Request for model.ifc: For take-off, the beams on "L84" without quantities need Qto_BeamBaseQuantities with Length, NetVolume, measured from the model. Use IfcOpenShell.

First a look at what the model holds.

```python
import ifcopenshell
import ifcopenshell.util.element
import ifcopenshell.util.unit

model = ifcopenshell.open("model.ifc")
print(model.schema)
for unit_type in ("LENGTHUNIT", "AREAUNIT", "VOLUMEUNIT"):
    print(unit_type, ifcopenshell.util.unit.calculate_unit_scale(model, unit_type))
storey = next(s for s in model.by_type("IfcBuildingStorey") if s.Name == "L84")
beams = [e for e in ifcopenshell.util.element.get_decomposition(storey) if e.is_a("IfcBeam")]
for e in sorted(beams, key=lambda e: e.id()):
    print(e.id(), e.is_a(), e.Name, list(ifcopenshell.util.element.get_psets(e, qtos_only=True)), sep=" | ")
```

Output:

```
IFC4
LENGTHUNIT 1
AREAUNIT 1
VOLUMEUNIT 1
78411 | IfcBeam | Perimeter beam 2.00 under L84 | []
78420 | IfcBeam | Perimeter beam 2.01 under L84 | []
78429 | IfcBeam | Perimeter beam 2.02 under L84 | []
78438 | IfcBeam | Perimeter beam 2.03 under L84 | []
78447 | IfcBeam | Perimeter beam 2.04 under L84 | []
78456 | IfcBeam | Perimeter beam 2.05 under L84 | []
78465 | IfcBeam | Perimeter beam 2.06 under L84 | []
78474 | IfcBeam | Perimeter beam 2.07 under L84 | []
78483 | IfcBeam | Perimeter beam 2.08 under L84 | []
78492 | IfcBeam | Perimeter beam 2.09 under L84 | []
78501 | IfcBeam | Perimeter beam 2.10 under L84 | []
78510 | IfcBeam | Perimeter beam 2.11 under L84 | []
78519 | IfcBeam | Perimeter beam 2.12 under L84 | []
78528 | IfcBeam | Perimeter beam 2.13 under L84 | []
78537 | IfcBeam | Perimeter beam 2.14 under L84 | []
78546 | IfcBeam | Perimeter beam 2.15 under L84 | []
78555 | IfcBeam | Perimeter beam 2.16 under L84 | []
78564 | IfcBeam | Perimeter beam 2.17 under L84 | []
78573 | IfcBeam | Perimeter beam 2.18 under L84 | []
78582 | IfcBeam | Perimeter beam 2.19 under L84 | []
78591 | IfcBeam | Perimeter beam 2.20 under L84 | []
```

```python
import ifcopenshell
import ifcopenshell.api.pset
import ifcopenshell.geom
import ifcopenshell.util.element
import ifcopenshell.util.shape
import ifcopenshell.util.unit

model = ifcopenshell.open("model.ifc")
unit_scale = ifcopenshell.util.unit.calculate_unit_scale(model)
volume_scale = ifcopenshell.util.unit.calculate_unit_scale(model, "VOLUMEUNIT")
settings = ifcopenshell.geom.settings()

storey = next(s for s in model.by_type("IfcBuildingStorey") if s.Name == "L84")
beams = [e for e in ifcopenshell.util.element.get_decomposition(storey) if e.is_a("IfcBeam")]

for e in sorted(beams, key=lambda e: e.id()):
    if ifcopenshell.util.element.get_psets(e, qtos_only=True, should_inherit=False):
        continue
    # Geometry comes back in metres, in the element's own axes.
    shape = ifcopenshell.geom.create_shape(settings, e)
    values = {
        "Length": ifcopenshell.util.shape.get_max_xyz(shape.geometry) / unit_scale,
        "NetVolume": ifcopenshell.util.shape.get_volume(shape.geometry) / volume_scale,
    }
    qto = ifcopenshell.api.pset.add_qto(model, product=e, name="Qto_BeamBaseQuantities")
    ifcopenshell.api.pset.edit_qto(model, qto=qto, properties=values)
    print(e.id(), {k: round(v, 3) for k, v in values.items()})

model.write("model_updated.ifc")
```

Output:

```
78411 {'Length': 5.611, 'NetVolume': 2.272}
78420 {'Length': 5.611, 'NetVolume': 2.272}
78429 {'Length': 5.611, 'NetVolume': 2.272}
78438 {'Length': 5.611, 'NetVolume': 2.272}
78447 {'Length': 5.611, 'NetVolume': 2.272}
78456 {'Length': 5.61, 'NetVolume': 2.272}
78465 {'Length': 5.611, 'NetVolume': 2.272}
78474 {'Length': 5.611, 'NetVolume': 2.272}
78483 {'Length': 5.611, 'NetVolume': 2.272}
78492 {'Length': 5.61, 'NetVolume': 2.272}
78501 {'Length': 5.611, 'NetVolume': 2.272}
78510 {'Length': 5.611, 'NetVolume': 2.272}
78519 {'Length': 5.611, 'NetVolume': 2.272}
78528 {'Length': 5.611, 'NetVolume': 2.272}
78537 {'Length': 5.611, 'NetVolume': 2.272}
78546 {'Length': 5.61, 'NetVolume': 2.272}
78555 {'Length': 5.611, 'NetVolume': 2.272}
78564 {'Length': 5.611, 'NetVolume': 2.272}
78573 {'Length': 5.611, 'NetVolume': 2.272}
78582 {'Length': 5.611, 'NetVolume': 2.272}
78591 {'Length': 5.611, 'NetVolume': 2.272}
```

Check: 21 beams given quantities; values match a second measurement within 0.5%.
